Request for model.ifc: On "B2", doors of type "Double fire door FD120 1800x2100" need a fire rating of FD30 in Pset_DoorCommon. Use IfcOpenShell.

First a look at what the model holds.

```python
import ifcopenshell
import ifcopenshell.util.element

model = ifcopenshell.open("model.ifc")
print(model.schema)
storey = next(s for s in model.by_type("IfcBuildingStorey") if s.Name == "B2")
doors = [e for e in ifcopenshell.util.element.get_decomposition(storey) if e.is_a("IfcDoor")]
seen = {}
for e in doors:
    element_type = ifcopenshell.util.element.get_type(e)
    key = (element_type.Name if element_type != e and element_type else None, ifcopenshell.util.element.get_pset(e, "Pset_DoorCommon", "FireRating"))
    seen[key] = seen.get(key, 0) + 1
for (name, value), count in sorted(seen.items(), key=str):
    print(count, "x", name, "|", value)
```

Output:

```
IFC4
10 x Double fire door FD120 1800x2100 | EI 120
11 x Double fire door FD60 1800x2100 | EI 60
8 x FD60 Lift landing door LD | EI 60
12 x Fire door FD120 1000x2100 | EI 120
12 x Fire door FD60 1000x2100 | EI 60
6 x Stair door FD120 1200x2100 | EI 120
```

```python
import ifcopenshell
import ifcopenshell.api.pset
import ifcopenshell.util.element

model = ifcopenshell.open("model.ifc")

storey = next(s for s in model.by_type("IfcBuildingStorey") if s.Name == "B2")
doors = [e for e in ifcopenshell.util.element.get_decomposition(storey) if e.is_a("IfcDoor")]

count = 0
for e in doors:
    element_type = ifcopenshell.util.element.get_type(e)
    if element_type in (None, e) or element_type.Name != "Double fire door FD120 1800x2100":
        continue
    # add_pset returns the element's existing set when there is one.
    pset = ifcopenshell.api.pset.add_pset(model, product=e, name="Pset_DoorCommon")
    ifcopenshell.api.pset.edit_pset(model, pset=pset, properties={"FireRating": "FD30"})
    count += 1

print(count, "doors updated")

model.write("model_updated.ifc")
```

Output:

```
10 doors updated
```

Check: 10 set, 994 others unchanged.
